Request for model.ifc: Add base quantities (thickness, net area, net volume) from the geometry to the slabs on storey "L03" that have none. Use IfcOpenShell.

First a look at what the model holds.

```python
import ifcopenshell
import ifcopenshell.util.element
import ifcopenshell.util.unit

model = ifcopenshell.open("model.ifc")
print(model.schema)
for unit_type in ("LENGTHUNIT", "AREAUNIT", "VOLUMEUNIT"):
    print(unit_type, ifcopenshell.util.unit.calculate_unit_scale(model, unit_type))
storey = next(s for s in model.by_type("IfcBuildingStorey") if s.Name == "L03")
slabs = [e for e in ifcopenshell.util.element.get_decomposition(storey) if e.is_a("IfcSlab")]
for e in sorted(slabs, key=lambda e: e.id()):
    print(e.id(), e.is_a(), e.Name, list(ifcopenshell.util.element.get_psets(e, qtos_only=True)), sep=" | ")
```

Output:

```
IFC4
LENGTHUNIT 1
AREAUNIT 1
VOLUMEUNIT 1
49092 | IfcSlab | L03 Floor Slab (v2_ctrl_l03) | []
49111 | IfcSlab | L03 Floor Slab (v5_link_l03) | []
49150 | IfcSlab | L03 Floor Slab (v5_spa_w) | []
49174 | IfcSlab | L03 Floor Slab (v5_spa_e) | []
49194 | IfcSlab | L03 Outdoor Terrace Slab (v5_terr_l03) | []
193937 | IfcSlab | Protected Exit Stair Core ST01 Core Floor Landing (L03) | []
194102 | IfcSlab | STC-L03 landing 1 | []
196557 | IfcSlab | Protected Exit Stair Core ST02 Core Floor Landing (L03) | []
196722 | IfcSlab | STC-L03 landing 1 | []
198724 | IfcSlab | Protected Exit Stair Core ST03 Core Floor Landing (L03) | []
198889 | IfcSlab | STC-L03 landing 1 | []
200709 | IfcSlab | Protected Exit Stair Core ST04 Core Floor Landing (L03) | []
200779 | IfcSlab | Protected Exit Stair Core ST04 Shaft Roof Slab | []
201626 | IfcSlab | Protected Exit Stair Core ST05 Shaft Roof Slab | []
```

```python
import ifcopenshell
import ifcopenshell.api.pset
import ifcopenshell.geom
import ifcopenshell.util.element
import ifcopenshell.util.shape
import ifcopenshell.util.unit

model = ifcopenshell.open("model.ifc")
unit_scale = ifcopenshell.util.unit.calculate_unit_scale(model)
area_scale = ifcopenshell.util.unit.calculate_unit_scale(model, "AREAUNIT")
volume_scale = ifcopenshell.util.unit.calculate_unit_scale(model, "VOLUMEUNIT")
settings = ifcopenshell.geom.settings()

storey = next(s for s in model.by_type("IfcBuildingStorey") if s.Name == "L03")
slabs = [e for e in ifcopenshell.util.element.get_decomposition(storey) if e.is_a("IfcSlab")]

for e in sorted(slabs, key=lambda e: e.id()):
    if ifcopenshell.util.element.get_psets(e, qtos_only=True, should_inherit=False):
        continue
    # Geometry comes back in metres, in the element's own axes.
    shape = ifcopenshell.geom.create_shape(settings, e)
    values = {
        "Width": ifcopenshell.util.shape.get_z(shape.geometry) / unit_scale,
        "NetArea": ifcopenshell.util.shape.get_footprint_area(shape.geometry) / area_scale,
        "NetVolume": ifcopenshell.util.shape.get_volume(shape.geometry) / volume_scale,
    }
    qto = ifcopenshell.api.pset.add_qto(model, product=e, name="Qto_SlabBaseQuantities")
    ifcopenshell.api.pset.edit_qto(model, qto=qto, properties=values)
    print(e.id(), {k: round(v, 3) for k, v in values.items()})

model.write("model-out.ifc")
```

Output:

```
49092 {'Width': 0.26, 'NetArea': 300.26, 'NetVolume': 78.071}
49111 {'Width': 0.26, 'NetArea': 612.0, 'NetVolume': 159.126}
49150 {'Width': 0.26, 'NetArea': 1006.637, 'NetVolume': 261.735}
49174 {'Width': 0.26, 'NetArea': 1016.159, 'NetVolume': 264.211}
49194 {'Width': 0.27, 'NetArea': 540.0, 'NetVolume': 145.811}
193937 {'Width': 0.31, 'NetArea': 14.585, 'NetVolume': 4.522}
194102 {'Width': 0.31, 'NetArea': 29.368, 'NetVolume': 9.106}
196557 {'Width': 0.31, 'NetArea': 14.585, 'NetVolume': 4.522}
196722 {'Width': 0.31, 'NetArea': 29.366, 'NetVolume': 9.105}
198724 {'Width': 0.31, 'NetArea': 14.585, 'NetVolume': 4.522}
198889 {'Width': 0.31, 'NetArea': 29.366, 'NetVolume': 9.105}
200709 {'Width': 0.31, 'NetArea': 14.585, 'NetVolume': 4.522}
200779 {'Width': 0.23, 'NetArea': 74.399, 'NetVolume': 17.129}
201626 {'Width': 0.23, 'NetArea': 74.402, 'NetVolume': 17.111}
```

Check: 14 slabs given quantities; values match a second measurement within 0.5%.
